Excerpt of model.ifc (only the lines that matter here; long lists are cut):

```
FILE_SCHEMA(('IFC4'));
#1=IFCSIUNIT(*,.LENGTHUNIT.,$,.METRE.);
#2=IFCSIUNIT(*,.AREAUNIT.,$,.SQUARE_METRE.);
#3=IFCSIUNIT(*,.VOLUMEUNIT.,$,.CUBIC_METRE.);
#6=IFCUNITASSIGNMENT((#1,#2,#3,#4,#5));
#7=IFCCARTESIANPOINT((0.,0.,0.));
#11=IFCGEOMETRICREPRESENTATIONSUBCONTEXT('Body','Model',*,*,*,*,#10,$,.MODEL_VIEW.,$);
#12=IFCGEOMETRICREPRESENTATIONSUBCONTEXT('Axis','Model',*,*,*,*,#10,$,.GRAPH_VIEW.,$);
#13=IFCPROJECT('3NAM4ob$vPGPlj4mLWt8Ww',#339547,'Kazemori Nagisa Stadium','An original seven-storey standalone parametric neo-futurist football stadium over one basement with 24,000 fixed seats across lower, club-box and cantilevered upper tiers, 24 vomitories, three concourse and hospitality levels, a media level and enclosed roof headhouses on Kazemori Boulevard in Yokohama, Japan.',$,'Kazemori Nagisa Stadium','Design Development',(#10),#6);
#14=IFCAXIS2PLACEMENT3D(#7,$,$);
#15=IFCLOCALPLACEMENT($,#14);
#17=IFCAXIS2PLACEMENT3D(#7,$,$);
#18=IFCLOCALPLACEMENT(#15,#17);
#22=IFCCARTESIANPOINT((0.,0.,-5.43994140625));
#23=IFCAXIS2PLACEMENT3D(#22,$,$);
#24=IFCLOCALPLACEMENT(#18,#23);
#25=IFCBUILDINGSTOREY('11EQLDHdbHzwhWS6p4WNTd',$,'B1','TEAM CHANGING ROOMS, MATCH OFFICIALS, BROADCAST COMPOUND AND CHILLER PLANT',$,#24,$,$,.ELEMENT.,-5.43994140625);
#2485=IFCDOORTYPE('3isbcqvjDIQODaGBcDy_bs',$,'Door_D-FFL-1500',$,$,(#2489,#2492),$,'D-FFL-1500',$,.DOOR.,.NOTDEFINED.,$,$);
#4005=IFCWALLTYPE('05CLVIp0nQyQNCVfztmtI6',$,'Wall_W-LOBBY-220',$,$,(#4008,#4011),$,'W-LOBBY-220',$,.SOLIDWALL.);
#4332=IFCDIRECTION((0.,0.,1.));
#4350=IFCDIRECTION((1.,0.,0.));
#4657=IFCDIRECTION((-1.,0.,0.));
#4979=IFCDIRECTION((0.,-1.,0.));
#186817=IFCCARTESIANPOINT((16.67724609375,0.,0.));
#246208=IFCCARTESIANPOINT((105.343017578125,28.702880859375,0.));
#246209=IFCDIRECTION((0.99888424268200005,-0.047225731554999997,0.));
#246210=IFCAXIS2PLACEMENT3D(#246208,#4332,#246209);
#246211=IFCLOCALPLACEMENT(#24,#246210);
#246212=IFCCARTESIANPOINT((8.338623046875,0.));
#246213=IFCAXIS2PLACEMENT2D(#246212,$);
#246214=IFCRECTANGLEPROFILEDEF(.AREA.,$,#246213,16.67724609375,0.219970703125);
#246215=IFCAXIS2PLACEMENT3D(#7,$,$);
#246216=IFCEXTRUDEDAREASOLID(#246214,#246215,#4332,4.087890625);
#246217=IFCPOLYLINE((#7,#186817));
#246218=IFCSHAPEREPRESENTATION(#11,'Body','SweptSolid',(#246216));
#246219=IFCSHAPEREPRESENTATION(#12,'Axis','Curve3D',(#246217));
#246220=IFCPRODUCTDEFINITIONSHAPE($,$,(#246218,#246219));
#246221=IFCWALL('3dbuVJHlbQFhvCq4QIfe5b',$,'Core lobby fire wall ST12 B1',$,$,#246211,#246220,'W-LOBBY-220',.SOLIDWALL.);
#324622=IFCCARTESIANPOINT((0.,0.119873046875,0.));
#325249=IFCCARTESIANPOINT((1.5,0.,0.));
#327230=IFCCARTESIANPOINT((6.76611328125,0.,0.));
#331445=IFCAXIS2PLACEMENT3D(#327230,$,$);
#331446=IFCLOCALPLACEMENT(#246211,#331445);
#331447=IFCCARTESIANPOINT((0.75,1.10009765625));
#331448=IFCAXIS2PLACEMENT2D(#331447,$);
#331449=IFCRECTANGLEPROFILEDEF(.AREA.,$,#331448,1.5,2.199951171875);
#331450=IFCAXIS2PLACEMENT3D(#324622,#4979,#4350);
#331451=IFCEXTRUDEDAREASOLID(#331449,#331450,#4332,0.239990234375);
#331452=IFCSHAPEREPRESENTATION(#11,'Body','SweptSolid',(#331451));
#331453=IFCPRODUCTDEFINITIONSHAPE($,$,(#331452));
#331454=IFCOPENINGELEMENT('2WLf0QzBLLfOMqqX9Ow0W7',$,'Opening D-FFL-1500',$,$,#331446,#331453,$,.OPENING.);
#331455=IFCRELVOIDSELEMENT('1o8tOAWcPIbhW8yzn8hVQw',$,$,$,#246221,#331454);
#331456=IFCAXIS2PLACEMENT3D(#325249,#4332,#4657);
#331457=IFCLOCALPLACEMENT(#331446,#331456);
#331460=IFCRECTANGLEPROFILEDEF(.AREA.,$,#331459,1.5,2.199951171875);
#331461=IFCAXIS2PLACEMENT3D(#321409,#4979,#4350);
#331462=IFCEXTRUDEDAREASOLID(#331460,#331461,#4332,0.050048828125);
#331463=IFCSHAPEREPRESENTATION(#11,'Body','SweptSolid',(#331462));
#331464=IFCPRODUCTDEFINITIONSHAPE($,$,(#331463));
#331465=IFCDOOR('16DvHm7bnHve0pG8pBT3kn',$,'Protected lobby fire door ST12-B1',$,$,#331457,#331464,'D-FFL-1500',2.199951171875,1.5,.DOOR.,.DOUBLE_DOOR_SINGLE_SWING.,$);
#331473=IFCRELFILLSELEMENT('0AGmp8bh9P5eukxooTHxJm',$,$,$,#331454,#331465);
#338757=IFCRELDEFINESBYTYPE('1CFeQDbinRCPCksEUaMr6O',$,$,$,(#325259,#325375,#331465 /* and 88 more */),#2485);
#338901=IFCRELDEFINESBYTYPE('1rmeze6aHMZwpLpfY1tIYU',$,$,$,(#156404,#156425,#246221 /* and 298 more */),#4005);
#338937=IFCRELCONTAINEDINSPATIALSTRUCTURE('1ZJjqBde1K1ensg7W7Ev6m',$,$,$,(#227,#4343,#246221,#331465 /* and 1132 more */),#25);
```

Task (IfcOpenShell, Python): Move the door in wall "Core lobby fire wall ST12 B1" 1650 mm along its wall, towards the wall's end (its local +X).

```python
import ifcopenshell
import ifcopenshell.api.geometry
import ifcopenshell.util.placement

model = ifcopenshell.open("model.ifc")

door = model.by_guid("16DvHm7bnHve0pG8pBT3kn")
opening = door.FillsVoids[0].RelatingOpeningElement
wall = opening.VoidsElements[0].RelatingBuildingElement

wall_matrix = ifcopenshell.util.placement.get_local_placement(wall.ObjectPlacement)
shift = wall_matrix[:3, 0] * 1.65
before = ifcopenshell.util.placement.get_local_placement(door.ObjectPlacement)[:3, 3].copy()

# The door is placed relative to its opening, so it follows when the opening moves.
matrix = ifcopenshell.util.placement.get_local_placement(opening.ObjectPlacement)
matrix[:3, 3] += shift
ifcopenshell.api.geometry.edit_object_placement(
    model, product=opening, matrix=matrix, is_si=False, should_transform_children=True
)

after = ifcopenshell.util.placement.get_local_placement(door.ObjectPlacement)[:3, 3]
print("door moved by", (after - before).round(3) + 0.0)

model.write("model_v2.ifc")
```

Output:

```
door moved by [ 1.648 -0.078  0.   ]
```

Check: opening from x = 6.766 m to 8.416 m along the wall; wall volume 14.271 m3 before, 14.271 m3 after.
